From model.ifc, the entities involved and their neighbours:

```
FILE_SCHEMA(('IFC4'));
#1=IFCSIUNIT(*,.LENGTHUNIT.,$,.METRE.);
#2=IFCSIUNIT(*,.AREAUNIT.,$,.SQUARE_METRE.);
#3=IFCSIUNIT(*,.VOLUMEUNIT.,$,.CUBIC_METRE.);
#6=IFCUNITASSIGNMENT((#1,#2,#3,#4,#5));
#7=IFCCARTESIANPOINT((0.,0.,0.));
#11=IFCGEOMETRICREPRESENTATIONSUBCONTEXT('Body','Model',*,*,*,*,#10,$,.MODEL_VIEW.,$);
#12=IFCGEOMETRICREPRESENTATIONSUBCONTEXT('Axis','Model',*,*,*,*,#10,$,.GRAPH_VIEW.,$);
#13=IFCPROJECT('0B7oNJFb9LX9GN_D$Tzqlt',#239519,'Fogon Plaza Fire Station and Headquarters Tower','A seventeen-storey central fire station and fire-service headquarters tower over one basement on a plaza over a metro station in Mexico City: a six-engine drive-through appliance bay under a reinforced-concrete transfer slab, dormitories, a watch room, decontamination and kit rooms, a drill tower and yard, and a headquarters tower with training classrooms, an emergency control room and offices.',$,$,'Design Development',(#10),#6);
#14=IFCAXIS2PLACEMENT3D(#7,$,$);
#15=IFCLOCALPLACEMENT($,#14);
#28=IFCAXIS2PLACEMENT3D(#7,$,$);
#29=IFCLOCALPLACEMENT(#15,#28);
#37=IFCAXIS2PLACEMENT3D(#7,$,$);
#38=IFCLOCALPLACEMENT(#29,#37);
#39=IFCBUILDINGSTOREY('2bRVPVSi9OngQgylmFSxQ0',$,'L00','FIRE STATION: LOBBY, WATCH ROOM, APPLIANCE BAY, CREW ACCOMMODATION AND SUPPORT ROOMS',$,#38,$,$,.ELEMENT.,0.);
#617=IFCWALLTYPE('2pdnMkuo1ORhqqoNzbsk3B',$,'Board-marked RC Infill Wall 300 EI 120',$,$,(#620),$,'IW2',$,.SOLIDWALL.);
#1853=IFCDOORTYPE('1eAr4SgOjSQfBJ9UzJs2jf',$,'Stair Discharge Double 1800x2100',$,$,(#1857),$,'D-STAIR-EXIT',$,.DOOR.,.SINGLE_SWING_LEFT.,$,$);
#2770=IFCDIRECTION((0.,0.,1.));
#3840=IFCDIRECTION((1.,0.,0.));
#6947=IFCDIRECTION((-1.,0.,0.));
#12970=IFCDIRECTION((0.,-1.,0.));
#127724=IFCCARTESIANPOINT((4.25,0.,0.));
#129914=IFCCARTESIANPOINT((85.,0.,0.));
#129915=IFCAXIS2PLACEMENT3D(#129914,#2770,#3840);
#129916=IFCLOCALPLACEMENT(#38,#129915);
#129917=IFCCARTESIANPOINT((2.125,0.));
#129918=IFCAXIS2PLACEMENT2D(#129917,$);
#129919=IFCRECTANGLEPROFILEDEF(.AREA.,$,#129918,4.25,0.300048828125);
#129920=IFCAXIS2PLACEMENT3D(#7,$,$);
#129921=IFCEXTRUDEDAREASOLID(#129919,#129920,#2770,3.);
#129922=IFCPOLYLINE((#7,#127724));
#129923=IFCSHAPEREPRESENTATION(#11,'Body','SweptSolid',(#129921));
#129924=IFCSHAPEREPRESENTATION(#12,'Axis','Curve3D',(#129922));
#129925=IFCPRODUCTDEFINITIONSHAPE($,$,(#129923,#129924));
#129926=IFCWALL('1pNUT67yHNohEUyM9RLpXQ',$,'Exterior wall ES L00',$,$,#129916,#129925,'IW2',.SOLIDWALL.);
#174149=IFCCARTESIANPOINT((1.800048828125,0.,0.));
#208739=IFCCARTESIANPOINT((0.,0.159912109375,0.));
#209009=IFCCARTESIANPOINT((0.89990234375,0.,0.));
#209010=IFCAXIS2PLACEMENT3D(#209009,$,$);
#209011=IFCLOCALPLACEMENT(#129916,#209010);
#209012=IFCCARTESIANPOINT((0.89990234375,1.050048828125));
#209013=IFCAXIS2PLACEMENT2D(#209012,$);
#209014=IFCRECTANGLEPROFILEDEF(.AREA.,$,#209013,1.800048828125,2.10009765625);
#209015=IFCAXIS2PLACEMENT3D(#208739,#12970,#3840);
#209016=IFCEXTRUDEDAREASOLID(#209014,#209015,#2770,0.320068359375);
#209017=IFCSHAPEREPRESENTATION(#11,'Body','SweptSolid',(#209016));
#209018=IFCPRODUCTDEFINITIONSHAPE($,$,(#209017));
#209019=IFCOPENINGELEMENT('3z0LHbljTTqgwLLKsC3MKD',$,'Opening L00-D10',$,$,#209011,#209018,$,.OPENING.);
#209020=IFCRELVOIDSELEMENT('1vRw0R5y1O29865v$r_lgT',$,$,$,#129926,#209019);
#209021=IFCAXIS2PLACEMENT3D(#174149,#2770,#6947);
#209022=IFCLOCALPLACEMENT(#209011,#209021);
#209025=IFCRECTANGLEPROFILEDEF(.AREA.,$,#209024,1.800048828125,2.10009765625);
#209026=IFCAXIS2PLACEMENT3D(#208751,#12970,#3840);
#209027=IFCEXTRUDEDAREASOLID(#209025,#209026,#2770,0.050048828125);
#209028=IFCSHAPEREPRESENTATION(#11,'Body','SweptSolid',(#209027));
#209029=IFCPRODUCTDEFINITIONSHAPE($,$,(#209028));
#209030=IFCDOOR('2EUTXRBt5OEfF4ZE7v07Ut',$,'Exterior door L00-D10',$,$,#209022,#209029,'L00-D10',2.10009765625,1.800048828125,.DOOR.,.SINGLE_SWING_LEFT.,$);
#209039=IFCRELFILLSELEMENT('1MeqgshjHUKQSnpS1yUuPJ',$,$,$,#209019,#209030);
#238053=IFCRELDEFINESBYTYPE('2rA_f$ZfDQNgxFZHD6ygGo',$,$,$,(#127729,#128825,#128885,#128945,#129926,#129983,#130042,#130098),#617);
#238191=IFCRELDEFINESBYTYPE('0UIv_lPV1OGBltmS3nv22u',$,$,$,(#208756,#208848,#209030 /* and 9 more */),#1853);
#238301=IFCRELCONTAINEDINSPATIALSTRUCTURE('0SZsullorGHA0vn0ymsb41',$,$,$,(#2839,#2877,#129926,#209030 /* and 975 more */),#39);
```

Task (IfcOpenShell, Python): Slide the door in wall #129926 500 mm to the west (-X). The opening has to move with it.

```python
import ifcopenshell
import ifcopenshell.api.geometry
import ifcopenshell.util.placement

model = ifcopenshell.open("model.ifc")

door = model.by_id(209030)
opening = door.FillsVoids[0].RelatingOpeningElement
wall = opening.VoidsElements[0].RelatingBuildingElement

wall_matrix = ifcopenshell.util.placement.get_local_placement(wall.ObjectPlacement)
shift = wall_matrix[:3, 0] * -0.5
before = ifcopenshell.util.placement.get_local_placement(door.ObjectPlacement)[:3, 3].copy()

# The door is placed relative to its opening, so it follows when the opening moves.
matrix = ifcopenshell.util.placement.get_local_placement(opening.ObjectPlacement)
matrix[:3, 3] += shift
ifcopenshell.api.geometry.edit_object_placement(
    model, product=opening, matrix=matrix, is_si=False, should_transform_children=True
)

after = ifcopenshell.util.placement.get_local_placement(door.ObjectPlacement)[:3, 3]
print("door moved by", (after - before).round(3) + 0.0)

model.write("model_rev.ifc")
```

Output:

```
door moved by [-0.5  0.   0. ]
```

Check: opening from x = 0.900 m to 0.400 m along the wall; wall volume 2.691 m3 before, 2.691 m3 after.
